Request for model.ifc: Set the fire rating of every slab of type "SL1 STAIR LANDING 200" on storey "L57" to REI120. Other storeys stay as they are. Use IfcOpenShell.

First a look at what the model holds.

```python
import ifcopenshell
import ifcopenshell.util.element

model = ifcopenshell.open("model.ifc")
print(model.schema)
storey = next(s for s in model.by_type("IfcBuildingStorey") if s.Name == "L57")
slabs = [e for e in ifcopenshell.util.element.get_decomposition(storey) if e.is_a("IfcSlab")]
seen = {}
for e in slabs:
    element_type = ifcopenshell.util.element.get_type(e)
    key = (element_type.Name if element_type != e and element_type else None, ifcopenshell.util.element.get_pset(e, "Pset_SlabCommon", "FireRating"))
    seen[key] = seen.get(key, 0) + 1
for (name, value), count in sorted(seen.items(), key=str):
    print(count, "x", name, "|", value)
```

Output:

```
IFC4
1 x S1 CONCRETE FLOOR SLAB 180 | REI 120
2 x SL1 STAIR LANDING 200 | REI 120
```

```python
import ifcopenshell
import ifcopenshell.api.pset
import ifcopenshell.util.element

model = ifcopenshell.open("model.ifc")

storey = next(s for s in model.by_type("IfcBuildingStorey") if s.Name == "L57")
slabs = [e for e in ifcopenshell.util.element.get_decomposition(storey) if e.is_a("IfcSlab")]

count = 0
for e in slabs:
    element_type = ifcopenshell.util.element.get_type(e)
    if element_type in (None, e) or element_type.Name != "SL1 STAIR LANDING 200":
        continue
    found = ifcopenshell.util.element.get_pset(e, "Pset_SlabCommon", should_inherit=False)
    if found:
        pset = model.by_id(found["id"])
        if len(ifcopenshell.util.element.get_elements_by_pset(pset)) > 1:
            pset = ifcopenshell.api.pset.unshare_pset(model, products=[e], pset=pset)[0]
    else:
        pset = ifcopenshell.api.pset.add_pset(model, product=e, name="Pset_SlabCommon")
    ifcopenshell.api.pset.edit_pset(model, pset=pset, properties={"FireRating": "REI120"})
    count += 1

print(count, "slabs updated")

model.write("model_updated.ifc")
```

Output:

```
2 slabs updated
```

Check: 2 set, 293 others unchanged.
